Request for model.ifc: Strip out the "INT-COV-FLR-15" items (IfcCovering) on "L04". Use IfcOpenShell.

First a look at what the model holds.

```python
import ifcopenshell
import ifcopenshell.util.element

model = ifcopenshell.open("model.ifc")
print(model.schema)
storey = next(s for s in model.by_type("IfcBuildingStorey") if s.Name == "L04")
coverings = [e for e in ifcopenshell.util.element.get_decomposition(storey) if e.is_a("IfcCovering")]
seen = {}
for e in coverings:
    element_type = ifcopenshell.util.element.get_type(e)
    name = element_type.Name if element_type not in (None, e) else None
    seen[name] = seen.get(name, 0) + 1
for name, count in sorted(seen.items(), key=str):
    print(count, "x", name)
```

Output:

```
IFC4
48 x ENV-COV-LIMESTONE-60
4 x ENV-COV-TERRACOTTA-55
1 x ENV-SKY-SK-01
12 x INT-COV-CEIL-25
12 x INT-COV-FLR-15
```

```python
import ifcopenshell
import ifcopenshell.api.root
import ifcopenshell.util.element

model = ifcopenshell.open("model.ifc")

storey = next(s for s in model.by_type("IfcBuildingStorey") if s.Name == "L04")
coverings = [e for e in ifcopenshell.util.element.get_decomposition(storey) if e.is_a("IfcCovering")]
targets = [e for e in coverings if (t := ifcopenshell.util.element.get_type(e)) not in (None, e) and t.Name == "INT-COV-FLR-15"]

for e in targets:
    ifcopenshell.api.root.remove_product(model, product=e)
print(len(targets), "removed")

model.write("model-out.ifc")
```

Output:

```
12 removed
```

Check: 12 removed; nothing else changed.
